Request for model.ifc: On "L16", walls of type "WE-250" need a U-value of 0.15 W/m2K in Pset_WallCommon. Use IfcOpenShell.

First a look at what the model holds.

```python
import ifcopenshell
import ifcopenshell.util.element

model = ifcopenshell.open("model.ifc")
print(model.schema)
storey = next(s for s in model.by_type("IfcBuildingStorey") if s.Name == "L16")
walls = [e for e in ifcopenshell.util.element.get_decomposition(storey) if e.is_a("IfcWall")]
seen = {}
for e in walls:
    element_type = ifcopenshell.util.element.get_type(e)
    key = (element_type.Name if element_type != e and element_type else None, ifcopenshell.util.element.get_pset(e, "Pset_WallCommon", "ThermalTransmittance"))
    seen[key] = seen.get(key, 0) + 1
for (name, value), count in sorted(seen.items(), key=str):
    print(count, "x", name, "|", value)
```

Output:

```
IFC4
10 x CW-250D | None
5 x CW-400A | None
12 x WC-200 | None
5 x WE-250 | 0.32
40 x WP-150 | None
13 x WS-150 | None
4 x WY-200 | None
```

```python
import ifcopenshell
import ifcopenshell.api.pset
import ifcopenshell.util.element

model = ifcopenshell.open("model.ifc")

storey = next(s for s in model.by_type("IfcBuildingStorey") if s.Name == "L16")
walls = [e for e in ifcopenshell.util.element.get_decomposition(storey) if e.is_a("IfcWall")]

count = 0
for e in walls:
    element_type = ifcopenshell.util.element.get_type(e)
    if element_type in (None, e) or element_type.Name != "WE-250":
        continue
    found = ifcopenshell.util.element.get_pset(e, "Pset_WallCommon", should_inherit=False)
    if found:
        pset = model.by_id(found["id"])
        if len(ifcopenshell.util.element.get_elements_by_pset(pset)) > 1:
            pset = ifcopenshell.api.pset.unshare_pset(model, products=[e], pset=pset)[0]
    else:
        pset = ifcopenshell.api.pset.add_pset(model, product=e, name="Pset_WallCommon")
    ifcopenshell.api.pset.edit_pset(model, pset=pset, properties={"ThermalTransmittance": 0.15})
    count += 1

print(count, "walls updated")

model.write("model-out.ifc")
```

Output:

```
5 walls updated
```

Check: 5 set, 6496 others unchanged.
